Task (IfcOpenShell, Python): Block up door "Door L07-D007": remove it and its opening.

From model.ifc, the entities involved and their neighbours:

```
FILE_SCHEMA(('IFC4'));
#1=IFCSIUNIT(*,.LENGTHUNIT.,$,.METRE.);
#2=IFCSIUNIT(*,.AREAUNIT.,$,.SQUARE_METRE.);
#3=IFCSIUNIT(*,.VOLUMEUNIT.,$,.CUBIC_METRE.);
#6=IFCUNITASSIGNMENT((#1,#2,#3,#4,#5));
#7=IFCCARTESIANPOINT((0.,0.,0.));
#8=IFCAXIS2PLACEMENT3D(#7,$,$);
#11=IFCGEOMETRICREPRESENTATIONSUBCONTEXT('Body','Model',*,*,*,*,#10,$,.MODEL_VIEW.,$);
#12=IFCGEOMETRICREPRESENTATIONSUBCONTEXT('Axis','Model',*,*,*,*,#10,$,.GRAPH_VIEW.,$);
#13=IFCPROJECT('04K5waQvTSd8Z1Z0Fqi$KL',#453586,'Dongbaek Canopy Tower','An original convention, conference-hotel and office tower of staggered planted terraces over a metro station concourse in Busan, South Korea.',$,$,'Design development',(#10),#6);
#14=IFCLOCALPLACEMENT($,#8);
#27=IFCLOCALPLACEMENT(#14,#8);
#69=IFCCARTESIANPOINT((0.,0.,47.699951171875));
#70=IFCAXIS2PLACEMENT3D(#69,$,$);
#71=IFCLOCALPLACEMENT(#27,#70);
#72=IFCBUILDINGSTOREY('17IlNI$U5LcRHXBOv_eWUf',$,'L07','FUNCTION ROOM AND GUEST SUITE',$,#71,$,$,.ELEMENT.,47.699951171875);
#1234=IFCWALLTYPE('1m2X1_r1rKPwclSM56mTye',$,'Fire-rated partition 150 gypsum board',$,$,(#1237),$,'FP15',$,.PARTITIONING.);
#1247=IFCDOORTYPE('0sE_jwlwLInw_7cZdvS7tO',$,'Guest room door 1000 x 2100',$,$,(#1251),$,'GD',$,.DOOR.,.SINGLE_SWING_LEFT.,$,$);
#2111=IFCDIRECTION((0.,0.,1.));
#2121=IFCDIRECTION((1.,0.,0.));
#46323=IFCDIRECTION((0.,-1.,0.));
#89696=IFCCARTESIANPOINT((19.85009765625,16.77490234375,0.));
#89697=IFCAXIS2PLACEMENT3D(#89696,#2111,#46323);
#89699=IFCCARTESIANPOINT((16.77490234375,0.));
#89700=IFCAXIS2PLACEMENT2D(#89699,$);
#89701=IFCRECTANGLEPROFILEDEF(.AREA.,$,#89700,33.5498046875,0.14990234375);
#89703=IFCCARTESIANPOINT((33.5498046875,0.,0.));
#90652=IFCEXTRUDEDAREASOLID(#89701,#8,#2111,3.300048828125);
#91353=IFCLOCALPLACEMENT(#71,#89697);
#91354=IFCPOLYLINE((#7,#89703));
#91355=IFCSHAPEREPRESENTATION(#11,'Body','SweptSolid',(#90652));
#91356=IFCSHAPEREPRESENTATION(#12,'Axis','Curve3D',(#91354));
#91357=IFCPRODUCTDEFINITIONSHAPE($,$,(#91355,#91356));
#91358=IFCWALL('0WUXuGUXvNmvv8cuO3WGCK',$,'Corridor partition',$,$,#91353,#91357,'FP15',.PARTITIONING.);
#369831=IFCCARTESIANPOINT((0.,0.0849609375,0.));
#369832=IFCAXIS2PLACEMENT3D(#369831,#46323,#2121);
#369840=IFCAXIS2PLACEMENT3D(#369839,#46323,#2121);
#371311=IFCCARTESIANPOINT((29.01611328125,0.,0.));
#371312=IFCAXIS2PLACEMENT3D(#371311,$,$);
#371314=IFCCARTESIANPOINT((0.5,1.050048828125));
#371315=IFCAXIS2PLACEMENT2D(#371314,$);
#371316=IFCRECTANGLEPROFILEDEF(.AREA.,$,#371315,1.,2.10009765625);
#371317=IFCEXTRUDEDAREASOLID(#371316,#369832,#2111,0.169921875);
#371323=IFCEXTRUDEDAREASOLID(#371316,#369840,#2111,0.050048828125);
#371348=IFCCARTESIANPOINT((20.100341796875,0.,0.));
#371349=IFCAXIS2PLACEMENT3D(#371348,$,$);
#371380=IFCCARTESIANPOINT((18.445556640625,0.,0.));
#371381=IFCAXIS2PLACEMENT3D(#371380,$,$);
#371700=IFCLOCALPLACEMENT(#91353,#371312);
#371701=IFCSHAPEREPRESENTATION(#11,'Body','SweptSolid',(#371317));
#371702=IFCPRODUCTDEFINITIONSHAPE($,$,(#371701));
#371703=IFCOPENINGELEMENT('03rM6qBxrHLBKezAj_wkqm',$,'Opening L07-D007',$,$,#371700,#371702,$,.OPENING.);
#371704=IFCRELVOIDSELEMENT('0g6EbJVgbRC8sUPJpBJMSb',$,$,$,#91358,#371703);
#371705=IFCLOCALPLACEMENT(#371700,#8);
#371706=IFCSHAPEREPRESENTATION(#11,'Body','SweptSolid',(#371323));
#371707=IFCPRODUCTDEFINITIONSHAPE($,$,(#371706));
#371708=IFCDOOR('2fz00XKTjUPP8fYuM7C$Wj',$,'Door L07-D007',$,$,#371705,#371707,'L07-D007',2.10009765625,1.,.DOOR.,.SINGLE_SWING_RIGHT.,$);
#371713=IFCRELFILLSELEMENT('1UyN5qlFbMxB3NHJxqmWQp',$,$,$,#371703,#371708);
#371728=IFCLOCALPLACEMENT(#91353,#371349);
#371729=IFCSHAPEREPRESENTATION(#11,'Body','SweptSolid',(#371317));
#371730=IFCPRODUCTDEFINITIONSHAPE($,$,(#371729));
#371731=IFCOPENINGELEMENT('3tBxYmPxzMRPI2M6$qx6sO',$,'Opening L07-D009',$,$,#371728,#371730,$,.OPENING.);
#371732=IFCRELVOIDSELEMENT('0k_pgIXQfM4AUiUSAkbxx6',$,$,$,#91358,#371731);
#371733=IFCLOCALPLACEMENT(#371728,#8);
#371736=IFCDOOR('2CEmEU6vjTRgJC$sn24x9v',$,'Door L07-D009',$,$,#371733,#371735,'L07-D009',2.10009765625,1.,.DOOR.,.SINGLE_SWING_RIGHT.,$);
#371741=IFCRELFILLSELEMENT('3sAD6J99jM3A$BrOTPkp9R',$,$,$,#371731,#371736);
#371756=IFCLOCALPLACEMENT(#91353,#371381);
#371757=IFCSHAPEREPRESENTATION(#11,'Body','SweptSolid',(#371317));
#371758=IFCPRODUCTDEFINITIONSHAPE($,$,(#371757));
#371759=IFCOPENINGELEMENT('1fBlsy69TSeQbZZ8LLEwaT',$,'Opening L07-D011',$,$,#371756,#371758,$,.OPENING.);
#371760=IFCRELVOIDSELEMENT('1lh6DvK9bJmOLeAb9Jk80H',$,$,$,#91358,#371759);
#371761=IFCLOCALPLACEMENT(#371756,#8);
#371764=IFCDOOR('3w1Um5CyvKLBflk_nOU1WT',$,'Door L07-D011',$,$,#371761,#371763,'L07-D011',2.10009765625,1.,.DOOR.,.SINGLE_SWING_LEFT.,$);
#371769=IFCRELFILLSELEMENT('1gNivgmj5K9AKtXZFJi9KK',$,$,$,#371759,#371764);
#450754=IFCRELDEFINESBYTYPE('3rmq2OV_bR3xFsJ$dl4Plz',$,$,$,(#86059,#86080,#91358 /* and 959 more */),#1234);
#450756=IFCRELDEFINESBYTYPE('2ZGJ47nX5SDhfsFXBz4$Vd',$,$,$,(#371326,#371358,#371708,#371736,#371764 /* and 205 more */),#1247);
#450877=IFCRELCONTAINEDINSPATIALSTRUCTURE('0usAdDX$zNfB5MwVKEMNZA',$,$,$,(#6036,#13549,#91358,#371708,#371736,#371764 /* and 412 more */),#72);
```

```python
import ifcopenshell
import ifcopenshell.api.feature
import ifcopenshell.api.root
import ifcopenshell.geom
import ifcopenshell.util.shape

model = ifcopenshell.open("model.ifc")
settings = ifcopenshell.geom.settings()


def volume(element):
    """Net volume in cubic metres, openings subtracted."""
    shape = ifcopenshell.geom.create_shape(settings, element)
    return ifcopenshell.util.shape.get_volume(shape.geometry)


door = model.by_id(371708)
opening = door.FillsVoids[0].RelatingOpeningElement
wall = opening.VoidsElements[0].RelatingBuildingElement
before = volume(wall)

ifcopenshell.api.root.remove_product(model, product=door)
ifcopenshell.api.feature.remove_feature(model, feature=opening)

after = volume(wall)

print(f"wall volume {before:.3f} -> {after:.3f} m3")

model.write("model_updated.ifc")
```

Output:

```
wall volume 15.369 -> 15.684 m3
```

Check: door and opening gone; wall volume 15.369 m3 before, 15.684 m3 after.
